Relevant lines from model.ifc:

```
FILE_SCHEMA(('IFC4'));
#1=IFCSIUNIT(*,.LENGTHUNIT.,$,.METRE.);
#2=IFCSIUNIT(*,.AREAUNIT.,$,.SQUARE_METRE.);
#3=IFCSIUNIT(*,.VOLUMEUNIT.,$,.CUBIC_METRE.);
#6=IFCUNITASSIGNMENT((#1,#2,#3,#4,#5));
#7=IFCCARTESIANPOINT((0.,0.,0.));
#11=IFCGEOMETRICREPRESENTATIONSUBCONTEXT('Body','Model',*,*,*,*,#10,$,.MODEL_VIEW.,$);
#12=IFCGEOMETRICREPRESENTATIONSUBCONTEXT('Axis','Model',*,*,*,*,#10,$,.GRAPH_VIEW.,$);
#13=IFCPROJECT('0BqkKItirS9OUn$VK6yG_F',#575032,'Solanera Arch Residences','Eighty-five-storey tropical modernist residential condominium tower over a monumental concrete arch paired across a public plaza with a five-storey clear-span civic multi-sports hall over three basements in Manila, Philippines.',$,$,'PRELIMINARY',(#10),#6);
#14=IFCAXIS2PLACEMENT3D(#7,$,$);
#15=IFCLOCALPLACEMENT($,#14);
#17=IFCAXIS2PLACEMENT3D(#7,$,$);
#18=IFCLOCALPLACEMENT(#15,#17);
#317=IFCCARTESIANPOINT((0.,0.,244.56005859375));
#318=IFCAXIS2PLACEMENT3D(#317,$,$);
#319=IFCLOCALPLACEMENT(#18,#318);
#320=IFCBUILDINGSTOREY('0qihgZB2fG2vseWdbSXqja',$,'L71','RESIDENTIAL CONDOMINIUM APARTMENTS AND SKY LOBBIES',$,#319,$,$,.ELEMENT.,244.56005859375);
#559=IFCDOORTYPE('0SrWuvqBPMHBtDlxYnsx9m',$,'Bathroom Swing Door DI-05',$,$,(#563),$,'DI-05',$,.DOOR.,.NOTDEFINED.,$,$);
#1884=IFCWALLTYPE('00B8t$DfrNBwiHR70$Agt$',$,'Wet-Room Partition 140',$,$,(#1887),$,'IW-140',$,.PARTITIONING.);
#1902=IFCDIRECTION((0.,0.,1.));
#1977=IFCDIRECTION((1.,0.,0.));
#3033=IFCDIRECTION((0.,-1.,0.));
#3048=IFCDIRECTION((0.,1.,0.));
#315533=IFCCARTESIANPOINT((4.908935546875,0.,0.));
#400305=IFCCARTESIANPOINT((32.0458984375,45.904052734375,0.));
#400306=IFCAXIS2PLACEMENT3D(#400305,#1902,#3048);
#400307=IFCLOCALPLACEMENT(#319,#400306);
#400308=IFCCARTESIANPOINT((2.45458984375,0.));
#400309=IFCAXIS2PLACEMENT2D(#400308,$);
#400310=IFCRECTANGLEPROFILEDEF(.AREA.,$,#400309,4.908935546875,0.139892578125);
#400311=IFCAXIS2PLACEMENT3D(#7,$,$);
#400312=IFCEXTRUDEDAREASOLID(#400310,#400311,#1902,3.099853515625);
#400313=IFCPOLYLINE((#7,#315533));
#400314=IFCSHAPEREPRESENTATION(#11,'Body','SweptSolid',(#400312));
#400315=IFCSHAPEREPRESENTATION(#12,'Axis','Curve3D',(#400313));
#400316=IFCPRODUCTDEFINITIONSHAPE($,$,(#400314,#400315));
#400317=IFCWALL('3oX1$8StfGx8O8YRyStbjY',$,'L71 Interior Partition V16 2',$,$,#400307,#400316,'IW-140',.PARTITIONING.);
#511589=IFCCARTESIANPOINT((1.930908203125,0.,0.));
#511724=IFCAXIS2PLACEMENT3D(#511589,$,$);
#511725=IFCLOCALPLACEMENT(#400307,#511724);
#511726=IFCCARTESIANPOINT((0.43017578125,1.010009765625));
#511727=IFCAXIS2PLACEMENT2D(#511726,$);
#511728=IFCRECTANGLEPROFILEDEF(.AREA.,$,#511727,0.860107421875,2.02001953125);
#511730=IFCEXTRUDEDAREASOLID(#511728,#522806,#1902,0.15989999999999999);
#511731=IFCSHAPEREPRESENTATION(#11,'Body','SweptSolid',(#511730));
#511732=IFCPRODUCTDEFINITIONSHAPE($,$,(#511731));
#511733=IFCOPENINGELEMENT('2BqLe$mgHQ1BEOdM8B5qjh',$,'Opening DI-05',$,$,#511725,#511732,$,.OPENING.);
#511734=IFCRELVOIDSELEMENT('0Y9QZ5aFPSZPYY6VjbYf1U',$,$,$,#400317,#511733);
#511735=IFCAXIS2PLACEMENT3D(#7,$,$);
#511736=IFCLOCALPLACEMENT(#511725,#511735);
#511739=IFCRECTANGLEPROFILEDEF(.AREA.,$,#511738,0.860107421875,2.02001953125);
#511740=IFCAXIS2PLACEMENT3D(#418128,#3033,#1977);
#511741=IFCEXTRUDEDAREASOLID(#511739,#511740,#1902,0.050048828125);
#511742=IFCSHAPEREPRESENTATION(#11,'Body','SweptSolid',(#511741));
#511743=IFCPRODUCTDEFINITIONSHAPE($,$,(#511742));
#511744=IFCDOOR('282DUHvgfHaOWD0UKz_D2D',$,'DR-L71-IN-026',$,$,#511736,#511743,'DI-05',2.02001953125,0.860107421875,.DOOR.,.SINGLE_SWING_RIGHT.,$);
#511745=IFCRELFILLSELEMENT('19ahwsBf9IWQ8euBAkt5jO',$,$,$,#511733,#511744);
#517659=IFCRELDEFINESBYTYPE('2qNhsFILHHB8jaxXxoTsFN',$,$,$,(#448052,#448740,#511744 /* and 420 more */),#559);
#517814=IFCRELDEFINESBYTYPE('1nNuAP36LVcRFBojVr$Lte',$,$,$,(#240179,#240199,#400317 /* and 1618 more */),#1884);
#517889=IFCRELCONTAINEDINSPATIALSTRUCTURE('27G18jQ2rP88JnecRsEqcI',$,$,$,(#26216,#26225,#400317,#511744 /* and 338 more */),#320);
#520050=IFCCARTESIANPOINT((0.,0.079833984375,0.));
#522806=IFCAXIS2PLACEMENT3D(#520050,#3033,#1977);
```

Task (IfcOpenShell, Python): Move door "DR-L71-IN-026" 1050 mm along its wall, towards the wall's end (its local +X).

```python
import ifcopenshell
import ifcopenshell.api.geometry
import ifcopenshell.util.placement
import ifcopenshell.util.unit

model = ifcopenshell.open("model.ifc")
unit_scale = ifcopenshell.util.unit.calculate_unit_scale(model)

door = model.by_id(511744)
opening = door.FillsVoids[0].RelatingOpeningElement
wall = opening.VoidsElements[0].RelatingBuildingElement

wall_matrix = ifcopenshell.util.placement.get_local_placement(wall.ObjectPlacement)
shift = wall_matrix[:3, 0] * 1.05 / unit_scale
before = ifcopenshell.util.placement.get_local_placement(door.ObjectPlacement)[:3, 3].copy()

# The door is placed relative to its opening, so it follows when the opening moves.
matrix = ifcopenshell.util.placement.get_local_placement(opening.ObjectPlacement)
matrix[:3, 3] += shift
ifcopenshell.api.geometry.edit_object_placement(
    model, product=opening, matrix=matrix, is_si=False, should_transform_children=True
)

after = ifcopenshell.util.placement.get_local_placement(door.ObjectPlacement)[:3, 3]
print("door moved by", (after - before).round(3) + 0.0)

model.write("model_updated.ifc")
```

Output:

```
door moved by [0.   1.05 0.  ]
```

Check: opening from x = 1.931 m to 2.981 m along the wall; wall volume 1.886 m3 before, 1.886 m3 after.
